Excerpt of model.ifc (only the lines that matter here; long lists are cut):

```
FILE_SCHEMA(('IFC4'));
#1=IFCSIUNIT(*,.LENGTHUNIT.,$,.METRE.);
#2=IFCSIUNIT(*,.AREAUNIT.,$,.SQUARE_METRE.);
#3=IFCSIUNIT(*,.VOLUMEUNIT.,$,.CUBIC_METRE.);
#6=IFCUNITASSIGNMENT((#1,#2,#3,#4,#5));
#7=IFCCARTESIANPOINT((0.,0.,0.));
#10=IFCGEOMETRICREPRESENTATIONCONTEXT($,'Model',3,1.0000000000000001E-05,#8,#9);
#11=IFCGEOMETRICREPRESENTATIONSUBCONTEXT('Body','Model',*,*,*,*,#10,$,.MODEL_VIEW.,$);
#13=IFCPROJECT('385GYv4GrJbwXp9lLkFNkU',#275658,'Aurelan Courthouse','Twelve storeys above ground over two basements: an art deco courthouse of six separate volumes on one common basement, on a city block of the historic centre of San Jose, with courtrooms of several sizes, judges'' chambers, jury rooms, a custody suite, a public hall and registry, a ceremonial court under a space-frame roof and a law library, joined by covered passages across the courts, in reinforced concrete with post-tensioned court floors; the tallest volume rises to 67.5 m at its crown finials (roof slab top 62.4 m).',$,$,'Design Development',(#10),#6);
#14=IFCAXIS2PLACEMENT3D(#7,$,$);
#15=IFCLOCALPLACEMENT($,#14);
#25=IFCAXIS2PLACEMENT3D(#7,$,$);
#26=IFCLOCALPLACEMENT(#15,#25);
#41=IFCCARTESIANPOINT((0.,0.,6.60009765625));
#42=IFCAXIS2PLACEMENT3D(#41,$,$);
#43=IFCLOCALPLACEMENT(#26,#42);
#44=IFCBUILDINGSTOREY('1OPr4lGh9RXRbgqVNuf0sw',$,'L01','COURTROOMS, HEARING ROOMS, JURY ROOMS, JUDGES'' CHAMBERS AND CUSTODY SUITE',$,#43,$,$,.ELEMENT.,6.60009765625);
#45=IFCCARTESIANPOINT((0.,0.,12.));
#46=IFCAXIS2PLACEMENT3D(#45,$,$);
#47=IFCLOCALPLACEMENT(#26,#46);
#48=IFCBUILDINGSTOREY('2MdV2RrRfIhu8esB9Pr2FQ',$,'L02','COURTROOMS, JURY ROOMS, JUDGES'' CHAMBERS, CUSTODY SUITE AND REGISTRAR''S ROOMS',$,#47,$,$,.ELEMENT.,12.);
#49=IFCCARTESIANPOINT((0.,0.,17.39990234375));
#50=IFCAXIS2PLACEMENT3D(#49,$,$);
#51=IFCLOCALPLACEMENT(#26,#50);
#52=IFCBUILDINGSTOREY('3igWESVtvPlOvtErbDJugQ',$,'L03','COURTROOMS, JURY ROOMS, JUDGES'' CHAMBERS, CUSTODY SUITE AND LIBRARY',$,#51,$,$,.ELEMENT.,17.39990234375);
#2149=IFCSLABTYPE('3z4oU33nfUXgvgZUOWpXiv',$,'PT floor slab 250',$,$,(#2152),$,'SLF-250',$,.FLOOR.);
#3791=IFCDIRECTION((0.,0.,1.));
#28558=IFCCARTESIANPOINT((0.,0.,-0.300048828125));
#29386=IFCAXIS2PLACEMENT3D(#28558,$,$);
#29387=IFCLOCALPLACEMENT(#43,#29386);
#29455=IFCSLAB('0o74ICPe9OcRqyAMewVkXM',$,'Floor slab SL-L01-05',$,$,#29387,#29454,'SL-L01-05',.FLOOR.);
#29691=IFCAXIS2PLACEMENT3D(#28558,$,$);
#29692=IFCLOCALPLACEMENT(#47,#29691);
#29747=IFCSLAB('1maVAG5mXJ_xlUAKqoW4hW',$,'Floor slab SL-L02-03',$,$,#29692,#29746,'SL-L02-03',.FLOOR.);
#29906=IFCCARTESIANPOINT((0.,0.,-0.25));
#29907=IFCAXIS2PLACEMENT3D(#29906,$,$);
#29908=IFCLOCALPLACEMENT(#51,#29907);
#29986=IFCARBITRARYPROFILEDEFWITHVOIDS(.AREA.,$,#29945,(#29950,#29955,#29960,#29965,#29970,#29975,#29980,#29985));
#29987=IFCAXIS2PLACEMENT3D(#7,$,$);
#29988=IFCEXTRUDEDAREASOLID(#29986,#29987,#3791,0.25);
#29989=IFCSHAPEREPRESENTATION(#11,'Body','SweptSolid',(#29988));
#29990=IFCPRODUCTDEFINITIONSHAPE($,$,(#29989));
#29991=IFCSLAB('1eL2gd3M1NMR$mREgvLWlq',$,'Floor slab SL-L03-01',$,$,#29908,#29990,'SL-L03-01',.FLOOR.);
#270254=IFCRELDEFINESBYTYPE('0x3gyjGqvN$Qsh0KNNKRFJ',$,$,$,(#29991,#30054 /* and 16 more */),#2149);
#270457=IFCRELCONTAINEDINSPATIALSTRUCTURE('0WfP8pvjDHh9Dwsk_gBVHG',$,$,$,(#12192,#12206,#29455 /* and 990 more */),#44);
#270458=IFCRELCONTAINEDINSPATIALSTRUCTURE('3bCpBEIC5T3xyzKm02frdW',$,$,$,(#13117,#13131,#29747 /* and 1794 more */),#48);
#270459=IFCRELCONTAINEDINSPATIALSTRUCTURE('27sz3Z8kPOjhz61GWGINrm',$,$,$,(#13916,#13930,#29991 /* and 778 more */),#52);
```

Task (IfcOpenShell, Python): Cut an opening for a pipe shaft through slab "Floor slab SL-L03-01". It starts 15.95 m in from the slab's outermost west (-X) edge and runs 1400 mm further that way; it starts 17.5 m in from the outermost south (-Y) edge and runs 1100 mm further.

```python
import numpy as np
import ifcopenshell
import ifcopenshell.api.feature
import ifcopenshell.api.geometry
import ifcopenshell.api.root
import ifcopenshell.geom
import ifcopenshell.util.placement
import ifcopenshell.util.representation
import ifcopenshell.util.shape
import ifcopenshell.util.unit

model = ifcopenshell.open("model.ifc")
unit_scale = ifcopenshell.util.unit.calculate_unit_scale(model)
settings = ifcopenshell.geom.settings()


def volume(element):
    """Net volume in cubic metres, openings subtracted."""
    shape = ifcopenshell.geom.create_shape(settings, element)
    return ifcopenshell.util.shape.get_volume(shape.geometry)


slab = model.by_id(29991)
before = volume(slab)

# Extent in the slab's own axes, in metres. The edges named are its -X and -Y sides.
slab_shape = ifcopenshell.geom.create_shape(settings, slab)
vertices = ifcopenshell.util.shape.get_vertices(slab_shape.geometry)
x_min, y_min, bottom = vertices.min(axis=0)
top = vertices[:, 2].max()

opening = ifcopenshell.api.root.create_entity(model, ifc_class="IfcOpeningElement", name="Pipe shaft opening", predefined_type="OPENING")
context = ifcopenshell.util.representation.get_context(model, "Model", "Body", "MODEL_VIEW")
width, depth = 1.4, 1.1
outline = [(0.0, 0.0), (width, 0.0), (width, depth), (0.0, depth), (0.0, 0.0)]
# Overshoot both faces by 50 mm so the cut is clean.
shape = ifcopenshell.api.geometry.add_slab_representation(
    model, context=context, depth=top - bottom + 0.1, polyline=outline
)
ifcopenshell.api.geometry.assign_representation(model, product=opening, representation=shape)

matrix = ifcopenshell.util.placement.get_local_placement(slab.ObjectPlacement)
matrix[:, 3] = matrix @ np.append(np.array([x_min + 15.95, y_min + 17.5, bottom - 0.05]) / unit_scale, 1.0)
ifcopenshell.api.geometry.edit_object_placement(model, product=opening, matrix=matrix, is_si=False)
ifcopenshell.api.feature.add_feature(model, feature=opening, element=slab)

after = volume(slab)

print(f"slab volume {before:.3f} -> {after:.3f} m3")

model.write("model_rev.ifc")
```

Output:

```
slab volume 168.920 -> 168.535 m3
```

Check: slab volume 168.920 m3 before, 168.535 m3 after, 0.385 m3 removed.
